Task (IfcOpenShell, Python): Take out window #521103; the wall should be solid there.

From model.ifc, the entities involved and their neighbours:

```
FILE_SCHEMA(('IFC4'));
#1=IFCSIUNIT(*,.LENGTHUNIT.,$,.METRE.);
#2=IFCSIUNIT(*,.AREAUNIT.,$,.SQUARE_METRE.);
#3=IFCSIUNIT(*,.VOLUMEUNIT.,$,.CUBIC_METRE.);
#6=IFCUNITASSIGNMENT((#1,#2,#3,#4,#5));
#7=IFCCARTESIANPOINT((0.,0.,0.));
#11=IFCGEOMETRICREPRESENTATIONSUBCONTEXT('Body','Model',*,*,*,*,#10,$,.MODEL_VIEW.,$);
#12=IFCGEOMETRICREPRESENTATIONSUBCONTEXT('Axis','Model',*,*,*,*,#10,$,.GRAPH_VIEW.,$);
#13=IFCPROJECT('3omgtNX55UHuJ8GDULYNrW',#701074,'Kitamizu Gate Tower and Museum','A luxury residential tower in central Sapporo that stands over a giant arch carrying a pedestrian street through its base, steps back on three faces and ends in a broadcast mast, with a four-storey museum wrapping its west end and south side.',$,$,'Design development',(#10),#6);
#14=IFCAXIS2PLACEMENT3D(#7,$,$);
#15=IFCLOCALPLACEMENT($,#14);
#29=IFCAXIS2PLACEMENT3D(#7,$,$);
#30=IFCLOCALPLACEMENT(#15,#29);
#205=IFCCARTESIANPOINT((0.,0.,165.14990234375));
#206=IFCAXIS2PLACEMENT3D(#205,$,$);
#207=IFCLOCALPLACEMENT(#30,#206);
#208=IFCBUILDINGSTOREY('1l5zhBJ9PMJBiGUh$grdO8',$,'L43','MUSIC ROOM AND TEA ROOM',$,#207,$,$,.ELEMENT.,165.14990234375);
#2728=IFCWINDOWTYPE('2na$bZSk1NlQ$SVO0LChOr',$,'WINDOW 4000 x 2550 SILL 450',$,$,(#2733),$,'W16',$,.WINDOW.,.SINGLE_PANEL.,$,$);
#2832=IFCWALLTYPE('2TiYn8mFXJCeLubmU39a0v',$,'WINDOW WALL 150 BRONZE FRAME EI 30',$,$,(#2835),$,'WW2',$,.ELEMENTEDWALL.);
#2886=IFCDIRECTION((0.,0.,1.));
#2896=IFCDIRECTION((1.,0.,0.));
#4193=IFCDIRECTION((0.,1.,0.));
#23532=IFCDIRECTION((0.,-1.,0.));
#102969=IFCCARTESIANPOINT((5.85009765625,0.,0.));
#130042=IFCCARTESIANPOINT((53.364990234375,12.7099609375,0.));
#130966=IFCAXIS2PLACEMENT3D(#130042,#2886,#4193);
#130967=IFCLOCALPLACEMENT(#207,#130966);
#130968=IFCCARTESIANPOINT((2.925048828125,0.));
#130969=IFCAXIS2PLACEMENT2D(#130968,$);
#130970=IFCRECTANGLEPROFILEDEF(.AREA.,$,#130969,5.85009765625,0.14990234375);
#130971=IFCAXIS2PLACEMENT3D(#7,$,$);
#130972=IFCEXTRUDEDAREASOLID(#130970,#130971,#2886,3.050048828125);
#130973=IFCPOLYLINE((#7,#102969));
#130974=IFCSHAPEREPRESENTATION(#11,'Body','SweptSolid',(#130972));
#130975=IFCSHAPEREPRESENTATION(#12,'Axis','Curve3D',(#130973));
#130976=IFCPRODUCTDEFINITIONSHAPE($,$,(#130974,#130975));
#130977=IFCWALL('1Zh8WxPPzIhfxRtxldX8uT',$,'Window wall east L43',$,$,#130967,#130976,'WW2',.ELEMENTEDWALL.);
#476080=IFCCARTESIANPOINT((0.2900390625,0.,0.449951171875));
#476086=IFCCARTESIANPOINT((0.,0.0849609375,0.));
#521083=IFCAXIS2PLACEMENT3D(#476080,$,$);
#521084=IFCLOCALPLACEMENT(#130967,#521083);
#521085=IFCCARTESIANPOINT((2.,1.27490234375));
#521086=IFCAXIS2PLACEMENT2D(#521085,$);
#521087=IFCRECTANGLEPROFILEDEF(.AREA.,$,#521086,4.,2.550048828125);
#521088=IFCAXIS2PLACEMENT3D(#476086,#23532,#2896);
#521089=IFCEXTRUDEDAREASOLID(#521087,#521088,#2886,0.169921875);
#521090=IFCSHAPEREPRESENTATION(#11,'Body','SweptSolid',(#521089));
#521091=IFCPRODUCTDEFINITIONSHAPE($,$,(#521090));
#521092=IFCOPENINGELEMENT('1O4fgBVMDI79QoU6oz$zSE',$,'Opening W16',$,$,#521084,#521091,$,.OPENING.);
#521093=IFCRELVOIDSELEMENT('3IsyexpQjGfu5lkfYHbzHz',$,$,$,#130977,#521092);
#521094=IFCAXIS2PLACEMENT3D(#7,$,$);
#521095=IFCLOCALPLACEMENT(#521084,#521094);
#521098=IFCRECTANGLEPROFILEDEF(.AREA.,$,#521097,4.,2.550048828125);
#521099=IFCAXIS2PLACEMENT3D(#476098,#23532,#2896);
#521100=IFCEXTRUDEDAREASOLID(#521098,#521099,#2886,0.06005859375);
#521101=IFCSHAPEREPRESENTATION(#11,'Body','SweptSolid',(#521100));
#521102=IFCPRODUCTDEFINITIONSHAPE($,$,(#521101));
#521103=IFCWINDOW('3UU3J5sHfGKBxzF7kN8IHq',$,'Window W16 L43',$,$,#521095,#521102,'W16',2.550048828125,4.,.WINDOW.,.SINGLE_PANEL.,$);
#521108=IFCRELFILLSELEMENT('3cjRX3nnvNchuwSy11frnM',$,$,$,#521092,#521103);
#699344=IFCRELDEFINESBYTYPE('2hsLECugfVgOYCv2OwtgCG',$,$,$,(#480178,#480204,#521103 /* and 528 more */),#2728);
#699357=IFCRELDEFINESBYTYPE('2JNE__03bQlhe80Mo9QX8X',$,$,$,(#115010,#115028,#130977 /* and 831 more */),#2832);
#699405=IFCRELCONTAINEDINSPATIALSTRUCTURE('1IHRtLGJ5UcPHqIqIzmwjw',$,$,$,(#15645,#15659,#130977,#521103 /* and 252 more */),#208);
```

```python
import ifcopenshell
import ifcopenshell.api.feature
import ifcopenshell.api.root
import ifcopenshell.geom
import ifcopenshell.util.shape

model = ifcopenshell.open("model.ifc")
settings = ifcopenshell.geom.settings()


def volume(element):
    """Net volume in cubic metres, openings subtracted."""
    shape = ifcopenshell.geom.create_shape(settings, element)
    return ifcopenshell.util.shape.get_volume(shape.geometry)


window = model.by_guid("3UU3J5sHfGKBxzF7kN8IHq")
opening = window.FillsVoids[0].RelatingOpeningElement
wall = opening.VoidsElements[0].RelatingBuildingElement
before = volume(wall)

ifcopenshell.api.root.remove_product(model, product=window)
ifcopenshell.api.feature.remove_feature(model, feature=opening)

after = volume(wall)

print(f"wall volume {before:.3f} -> {after:.3f} m3")

model.write("model-out.ifc")
```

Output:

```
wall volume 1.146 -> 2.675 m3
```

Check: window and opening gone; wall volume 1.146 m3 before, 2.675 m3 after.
